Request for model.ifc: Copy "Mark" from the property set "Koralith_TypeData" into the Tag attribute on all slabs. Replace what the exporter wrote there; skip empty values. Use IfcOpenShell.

First a look at what the model holds.

```python
import ifcopenshell
import ifcopenshell.util.element

model = ifcopenshell.open("model.ifc")
print(model.schema)
slabs = model.by_type("IfcSlab")
print(len(slabs), "slabs")
for e in slabs[:8]:
    source = ifcopenshell.util.element.get_pset(e, "Koralith_TypeData", "Mark")
    target = e.Tag
    print(e.id(), repr(source), repr(target), sep=" | ")
```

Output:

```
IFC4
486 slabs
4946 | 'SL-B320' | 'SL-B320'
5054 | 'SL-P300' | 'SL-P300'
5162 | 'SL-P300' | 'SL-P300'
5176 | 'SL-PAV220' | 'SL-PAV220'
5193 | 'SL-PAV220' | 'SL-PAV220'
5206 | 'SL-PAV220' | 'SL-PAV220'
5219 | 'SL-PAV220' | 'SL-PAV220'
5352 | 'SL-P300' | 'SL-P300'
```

```python
import ifcopenshell
import ifcopenshell.util.element

model = ifcopenshell.open("model.ifc")

count = 0
for e in model.by_type("IfcSlab"):
    value = ifcopenshell.util.element.get_pset(e, "Koralith_TypeData", "Mark")
    current = e.Tag
    if not value or not value.strip() or current == value:
        continue
    e.Tag = value
    count += 1

print(count, "slabs updated")

model.write("model_v2.ifc")
```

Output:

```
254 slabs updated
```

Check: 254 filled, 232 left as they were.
